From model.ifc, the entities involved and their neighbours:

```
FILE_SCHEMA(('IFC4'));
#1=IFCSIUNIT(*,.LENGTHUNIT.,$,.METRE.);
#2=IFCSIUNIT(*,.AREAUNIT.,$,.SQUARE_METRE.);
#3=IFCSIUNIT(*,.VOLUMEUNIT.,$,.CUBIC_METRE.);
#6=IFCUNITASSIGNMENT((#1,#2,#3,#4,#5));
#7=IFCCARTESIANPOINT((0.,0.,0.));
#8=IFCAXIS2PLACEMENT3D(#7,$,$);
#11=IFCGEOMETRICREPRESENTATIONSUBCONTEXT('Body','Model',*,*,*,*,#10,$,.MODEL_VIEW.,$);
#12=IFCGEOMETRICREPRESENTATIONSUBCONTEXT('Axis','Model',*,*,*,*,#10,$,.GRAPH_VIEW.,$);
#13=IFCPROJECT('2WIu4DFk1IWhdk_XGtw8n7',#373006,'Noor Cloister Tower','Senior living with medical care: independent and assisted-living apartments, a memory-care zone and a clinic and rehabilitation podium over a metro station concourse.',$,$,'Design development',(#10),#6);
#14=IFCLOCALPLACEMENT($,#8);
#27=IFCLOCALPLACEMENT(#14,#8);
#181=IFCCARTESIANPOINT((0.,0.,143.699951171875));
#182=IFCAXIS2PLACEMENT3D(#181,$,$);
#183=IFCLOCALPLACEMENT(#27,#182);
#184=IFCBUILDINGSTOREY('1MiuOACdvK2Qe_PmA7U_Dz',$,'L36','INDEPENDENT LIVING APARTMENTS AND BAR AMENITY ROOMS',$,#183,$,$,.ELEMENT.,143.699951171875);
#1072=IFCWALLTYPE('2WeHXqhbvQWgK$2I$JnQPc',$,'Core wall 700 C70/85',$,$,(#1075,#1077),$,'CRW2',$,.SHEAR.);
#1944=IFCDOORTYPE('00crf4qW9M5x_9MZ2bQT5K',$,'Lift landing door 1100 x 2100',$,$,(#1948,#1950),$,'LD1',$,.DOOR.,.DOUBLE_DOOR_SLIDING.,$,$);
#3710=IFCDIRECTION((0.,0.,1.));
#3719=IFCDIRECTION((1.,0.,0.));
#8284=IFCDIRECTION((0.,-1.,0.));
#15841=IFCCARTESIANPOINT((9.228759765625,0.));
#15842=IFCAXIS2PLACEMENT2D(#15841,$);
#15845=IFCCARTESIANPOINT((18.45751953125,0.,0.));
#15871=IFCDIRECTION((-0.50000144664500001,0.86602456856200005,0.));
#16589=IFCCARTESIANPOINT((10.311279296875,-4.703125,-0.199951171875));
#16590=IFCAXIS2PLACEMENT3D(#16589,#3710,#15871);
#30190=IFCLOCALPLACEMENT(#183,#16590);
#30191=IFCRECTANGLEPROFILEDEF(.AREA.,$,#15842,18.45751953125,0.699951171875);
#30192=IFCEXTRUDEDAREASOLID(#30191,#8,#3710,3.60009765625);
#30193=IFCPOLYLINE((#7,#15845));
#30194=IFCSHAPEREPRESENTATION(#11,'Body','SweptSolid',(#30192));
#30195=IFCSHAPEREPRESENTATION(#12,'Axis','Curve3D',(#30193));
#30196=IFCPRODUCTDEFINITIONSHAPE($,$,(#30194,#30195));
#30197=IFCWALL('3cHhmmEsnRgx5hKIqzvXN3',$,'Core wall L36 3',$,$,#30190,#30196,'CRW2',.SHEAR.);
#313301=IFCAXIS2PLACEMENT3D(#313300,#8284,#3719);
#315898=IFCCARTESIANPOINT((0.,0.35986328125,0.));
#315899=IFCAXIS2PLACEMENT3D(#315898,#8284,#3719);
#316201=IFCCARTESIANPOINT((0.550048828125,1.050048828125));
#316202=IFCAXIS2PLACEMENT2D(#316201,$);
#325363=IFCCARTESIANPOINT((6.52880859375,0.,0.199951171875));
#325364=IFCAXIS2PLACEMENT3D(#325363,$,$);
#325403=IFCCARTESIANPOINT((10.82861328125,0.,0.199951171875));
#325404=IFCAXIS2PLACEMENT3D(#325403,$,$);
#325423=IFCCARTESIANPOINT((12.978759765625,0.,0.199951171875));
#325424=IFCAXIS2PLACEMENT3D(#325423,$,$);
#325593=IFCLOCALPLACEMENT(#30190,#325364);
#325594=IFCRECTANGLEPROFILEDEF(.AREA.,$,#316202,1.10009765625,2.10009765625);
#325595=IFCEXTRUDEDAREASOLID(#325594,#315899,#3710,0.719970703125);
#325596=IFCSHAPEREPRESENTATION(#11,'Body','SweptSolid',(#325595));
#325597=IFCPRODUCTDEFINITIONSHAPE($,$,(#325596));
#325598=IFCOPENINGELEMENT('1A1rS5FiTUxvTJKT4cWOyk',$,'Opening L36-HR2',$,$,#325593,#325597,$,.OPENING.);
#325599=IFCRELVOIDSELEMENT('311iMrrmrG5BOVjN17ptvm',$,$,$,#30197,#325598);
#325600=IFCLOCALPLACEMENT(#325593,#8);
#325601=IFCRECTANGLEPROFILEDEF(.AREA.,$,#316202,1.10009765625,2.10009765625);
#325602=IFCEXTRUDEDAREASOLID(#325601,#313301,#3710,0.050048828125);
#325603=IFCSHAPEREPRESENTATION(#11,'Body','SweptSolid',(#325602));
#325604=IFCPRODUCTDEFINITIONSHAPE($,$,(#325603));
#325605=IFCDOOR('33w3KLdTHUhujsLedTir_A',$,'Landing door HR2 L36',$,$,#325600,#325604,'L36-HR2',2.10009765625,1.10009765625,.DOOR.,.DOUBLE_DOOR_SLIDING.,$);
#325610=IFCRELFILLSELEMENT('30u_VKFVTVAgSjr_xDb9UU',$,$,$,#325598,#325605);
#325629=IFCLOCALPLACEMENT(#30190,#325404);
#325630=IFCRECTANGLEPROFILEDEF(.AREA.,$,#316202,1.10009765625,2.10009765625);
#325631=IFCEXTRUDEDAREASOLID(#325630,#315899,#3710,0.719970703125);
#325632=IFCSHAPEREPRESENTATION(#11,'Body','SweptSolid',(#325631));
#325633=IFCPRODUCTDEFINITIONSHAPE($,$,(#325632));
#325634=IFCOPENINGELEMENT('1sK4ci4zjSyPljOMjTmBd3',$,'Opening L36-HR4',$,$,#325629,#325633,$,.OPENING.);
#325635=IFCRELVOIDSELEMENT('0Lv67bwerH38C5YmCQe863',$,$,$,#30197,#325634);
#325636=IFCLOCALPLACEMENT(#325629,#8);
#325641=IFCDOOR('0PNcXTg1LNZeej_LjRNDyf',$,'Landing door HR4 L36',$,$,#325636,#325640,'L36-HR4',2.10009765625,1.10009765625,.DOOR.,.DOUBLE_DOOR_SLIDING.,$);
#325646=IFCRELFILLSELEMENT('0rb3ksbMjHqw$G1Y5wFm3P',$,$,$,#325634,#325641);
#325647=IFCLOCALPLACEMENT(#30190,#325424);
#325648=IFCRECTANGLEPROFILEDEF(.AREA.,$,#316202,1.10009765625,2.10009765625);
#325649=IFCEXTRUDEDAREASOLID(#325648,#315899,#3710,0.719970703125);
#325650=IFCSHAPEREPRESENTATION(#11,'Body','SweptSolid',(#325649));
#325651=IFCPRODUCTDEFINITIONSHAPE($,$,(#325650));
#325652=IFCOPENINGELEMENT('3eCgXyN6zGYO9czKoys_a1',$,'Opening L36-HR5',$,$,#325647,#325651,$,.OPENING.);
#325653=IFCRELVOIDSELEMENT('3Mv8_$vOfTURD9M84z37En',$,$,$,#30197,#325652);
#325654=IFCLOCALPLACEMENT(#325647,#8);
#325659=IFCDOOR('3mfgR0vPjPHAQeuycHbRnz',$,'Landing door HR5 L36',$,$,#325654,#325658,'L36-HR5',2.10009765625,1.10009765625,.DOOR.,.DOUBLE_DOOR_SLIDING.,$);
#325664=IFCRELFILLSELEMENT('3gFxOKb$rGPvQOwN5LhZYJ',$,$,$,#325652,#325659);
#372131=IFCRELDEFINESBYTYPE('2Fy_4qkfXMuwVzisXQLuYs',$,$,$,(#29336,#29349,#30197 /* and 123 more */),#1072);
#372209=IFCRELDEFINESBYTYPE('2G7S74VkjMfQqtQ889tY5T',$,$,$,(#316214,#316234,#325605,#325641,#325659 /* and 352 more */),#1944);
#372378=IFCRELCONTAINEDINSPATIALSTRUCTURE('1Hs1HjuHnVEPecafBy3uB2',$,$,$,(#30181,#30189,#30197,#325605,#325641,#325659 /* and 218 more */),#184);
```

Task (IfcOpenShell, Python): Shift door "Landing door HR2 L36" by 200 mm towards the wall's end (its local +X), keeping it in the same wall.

```python
import ifcopenshell
import ifcopenshell.api.geometry
import ifcopenshell.util.placement
import ifcopenshell.util.unit

model = ifcopenshell.open("model.ifc")
unit_scale = ifcopenshell.util.unit.calculate_unit_scale(model)

door = model.by_guid("33w3KLdTHUhujsLedTir_A")
opening = door.FillsVoids[0].RelatingOpeningElement
wall = opening.VoidsElements[0].RelatingBuildingElement

wall_matrix = ifcopenshell.util.placement.get_local_placement(wall.ObjectPlacement)
shift = wall_matrix[:3, 0] * 0.2 / unit_scale
before = ifcopenshell.util.placement.get_local_placement(door.ObjectPlacement)[:3, 3].copy()

# The door is placed relative to its opening, so it follows when the opening moves.
matrix = ifcopenshell.util.placement.get_local_placement(opening.ObjectPlacement)
matrix[:3, 3] += shift
ifcopenshell.api.geometry.edit_object_placement(
    model, product=opening, matrix=matrix, is_si=False, should_transform_children=True
)

after = ifcopenshell.util.placement.get_local_placement(door.ObjectPlacement)[:3, 3]
print("door moved by", (after - before).round(3) + 0.0)

model.write("model-out.ifc")
```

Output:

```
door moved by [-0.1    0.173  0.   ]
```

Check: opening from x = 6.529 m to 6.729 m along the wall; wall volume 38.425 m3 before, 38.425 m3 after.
